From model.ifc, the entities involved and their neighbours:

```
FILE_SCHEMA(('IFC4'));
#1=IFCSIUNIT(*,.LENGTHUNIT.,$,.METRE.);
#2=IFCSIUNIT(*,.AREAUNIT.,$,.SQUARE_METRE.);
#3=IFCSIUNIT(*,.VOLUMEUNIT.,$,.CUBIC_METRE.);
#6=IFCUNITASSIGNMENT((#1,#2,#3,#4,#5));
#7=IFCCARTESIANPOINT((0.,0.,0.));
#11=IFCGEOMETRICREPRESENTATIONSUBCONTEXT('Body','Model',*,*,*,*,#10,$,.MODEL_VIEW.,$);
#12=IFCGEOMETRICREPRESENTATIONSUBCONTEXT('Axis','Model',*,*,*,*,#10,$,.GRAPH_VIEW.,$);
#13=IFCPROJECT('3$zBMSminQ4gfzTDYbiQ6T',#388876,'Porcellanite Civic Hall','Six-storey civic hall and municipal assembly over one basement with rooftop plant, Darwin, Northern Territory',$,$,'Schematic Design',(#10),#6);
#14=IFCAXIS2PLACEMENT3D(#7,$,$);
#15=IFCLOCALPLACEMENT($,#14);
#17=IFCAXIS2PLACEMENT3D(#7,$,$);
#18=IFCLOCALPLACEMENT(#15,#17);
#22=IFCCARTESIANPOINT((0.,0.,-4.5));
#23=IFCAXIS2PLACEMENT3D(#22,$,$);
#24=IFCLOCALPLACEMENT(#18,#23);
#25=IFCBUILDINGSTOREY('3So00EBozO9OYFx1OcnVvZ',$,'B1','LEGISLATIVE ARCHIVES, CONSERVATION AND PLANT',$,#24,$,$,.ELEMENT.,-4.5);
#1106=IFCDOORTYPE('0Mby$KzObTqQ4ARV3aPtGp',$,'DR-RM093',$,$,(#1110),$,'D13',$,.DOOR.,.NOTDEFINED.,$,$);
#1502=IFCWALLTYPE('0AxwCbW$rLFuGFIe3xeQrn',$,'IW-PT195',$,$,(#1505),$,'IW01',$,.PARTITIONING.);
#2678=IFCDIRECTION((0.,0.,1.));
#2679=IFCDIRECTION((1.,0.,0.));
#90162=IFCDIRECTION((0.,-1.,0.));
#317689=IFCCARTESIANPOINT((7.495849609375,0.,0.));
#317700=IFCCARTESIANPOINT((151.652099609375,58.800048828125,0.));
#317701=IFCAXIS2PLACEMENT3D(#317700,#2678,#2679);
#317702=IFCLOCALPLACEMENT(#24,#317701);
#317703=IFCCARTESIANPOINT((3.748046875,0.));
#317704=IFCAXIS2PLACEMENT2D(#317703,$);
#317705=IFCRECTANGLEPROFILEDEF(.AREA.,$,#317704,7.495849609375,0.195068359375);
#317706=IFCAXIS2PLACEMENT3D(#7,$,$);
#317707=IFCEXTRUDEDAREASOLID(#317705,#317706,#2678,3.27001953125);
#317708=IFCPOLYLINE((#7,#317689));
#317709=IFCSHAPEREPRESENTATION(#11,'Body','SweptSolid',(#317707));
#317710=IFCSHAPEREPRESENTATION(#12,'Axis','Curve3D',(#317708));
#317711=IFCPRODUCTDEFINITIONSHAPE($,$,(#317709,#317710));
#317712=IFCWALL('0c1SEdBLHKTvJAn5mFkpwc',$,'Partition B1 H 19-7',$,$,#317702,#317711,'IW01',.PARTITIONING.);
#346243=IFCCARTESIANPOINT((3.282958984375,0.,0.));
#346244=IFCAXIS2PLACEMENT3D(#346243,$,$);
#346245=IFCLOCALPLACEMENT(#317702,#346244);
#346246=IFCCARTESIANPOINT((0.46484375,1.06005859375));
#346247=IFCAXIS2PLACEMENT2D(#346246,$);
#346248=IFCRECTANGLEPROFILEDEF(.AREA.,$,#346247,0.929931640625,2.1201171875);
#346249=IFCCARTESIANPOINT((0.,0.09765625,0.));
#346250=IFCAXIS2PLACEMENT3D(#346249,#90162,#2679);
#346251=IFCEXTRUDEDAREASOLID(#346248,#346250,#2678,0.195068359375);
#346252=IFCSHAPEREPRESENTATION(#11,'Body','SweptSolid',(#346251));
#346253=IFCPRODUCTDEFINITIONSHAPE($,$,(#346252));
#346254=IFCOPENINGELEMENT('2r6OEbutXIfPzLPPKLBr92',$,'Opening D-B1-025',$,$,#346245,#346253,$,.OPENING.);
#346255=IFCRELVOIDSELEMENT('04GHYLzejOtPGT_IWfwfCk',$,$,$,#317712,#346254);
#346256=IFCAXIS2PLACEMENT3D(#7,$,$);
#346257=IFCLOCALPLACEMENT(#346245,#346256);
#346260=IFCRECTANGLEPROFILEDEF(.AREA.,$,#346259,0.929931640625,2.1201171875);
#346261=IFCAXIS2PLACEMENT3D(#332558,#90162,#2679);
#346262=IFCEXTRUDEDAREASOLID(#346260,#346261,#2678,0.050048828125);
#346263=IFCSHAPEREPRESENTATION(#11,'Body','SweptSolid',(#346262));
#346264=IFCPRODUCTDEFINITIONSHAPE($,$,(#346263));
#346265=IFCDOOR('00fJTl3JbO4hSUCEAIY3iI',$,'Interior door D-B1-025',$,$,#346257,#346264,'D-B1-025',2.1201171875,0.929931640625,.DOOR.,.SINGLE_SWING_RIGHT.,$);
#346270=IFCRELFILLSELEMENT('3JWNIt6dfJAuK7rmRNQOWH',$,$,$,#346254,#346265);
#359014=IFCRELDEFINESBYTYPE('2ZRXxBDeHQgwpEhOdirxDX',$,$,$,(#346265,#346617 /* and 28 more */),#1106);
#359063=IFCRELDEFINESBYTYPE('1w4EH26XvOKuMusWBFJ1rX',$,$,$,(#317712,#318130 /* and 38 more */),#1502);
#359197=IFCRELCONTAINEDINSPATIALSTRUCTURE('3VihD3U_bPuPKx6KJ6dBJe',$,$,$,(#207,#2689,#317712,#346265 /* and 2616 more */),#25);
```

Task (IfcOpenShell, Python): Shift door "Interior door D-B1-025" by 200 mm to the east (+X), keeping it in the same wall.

```python
import ifcopenshell
import ifcopenshell.api.geometry
import ifcopenshell.util.placement

model = ifcopenshell.open("model.ifc")

door = model.by_guid("00fJTl3JbO4hSUCEAIY3iI")
opening = door.FillsVoids[0].RelatingOpeningElement
wall = opening.VoidsElements[0].RelatingBuildingElement

wall_matrix = ifcopenshell.util.placement.get_local_placement(wall.ObjectPlacement)
shift = wall_matrix[:3, 0] * 0.2
before = ifcopenshell.util.placement.get_local_placement(door.ObjectPlacement)[:3, 3].copy()

# The door is placed relative to its opening, so it follows when the opening moves.
matrix = ifcopenshell.util.placement.get_local_placement(opening.ObjectPlacement)
matrix[:3, 3] += shift
ifcopenshell.api.geometry.edit_object_placement(
    model, product=opening, matrix=matrix, is_si=False, should_transform_children=True
)

after = ifcopenshell.util.placement.get_local_placement(door.ObjectPlacement)[:3, 3]
print("door moved by", (after - before).round(3) + 0.0)

model.write("model-out.ifc")
```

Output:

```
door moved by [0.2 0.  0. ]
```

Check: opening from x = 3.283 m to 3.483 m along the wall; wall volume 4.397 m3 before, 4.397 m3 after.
